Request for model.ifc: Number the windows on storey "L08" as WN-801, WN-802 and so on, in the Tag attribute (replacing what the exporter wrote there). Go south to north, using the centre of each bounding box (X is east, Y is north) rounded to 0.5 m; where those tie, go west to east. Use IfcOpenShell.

First a look at what the model holds.

```python
import ifcopenshell
import ifcopenshell.util.element
import ifcopenshell.util.placement

model = ifcopenshell.open("model.ifc")
print(model.schema)
storey = next(s for s in model.by_type("IfcBuildingStorey") if s.Name == "L08")
windows = [e for e in ifcopenshell.util.element.get_decomposition(storey) if e.is_a("IfcWindow")]
for e in sorted(windows, key=lambda e: e.id()):
    origin = ifcopenshell.util.placement.get_local_placement(e.ObjectPlacement)[:3, 3]
    print(e.id(), e.Tag, e.Name, origin.round(2) + 0.0, sep=" | ")
```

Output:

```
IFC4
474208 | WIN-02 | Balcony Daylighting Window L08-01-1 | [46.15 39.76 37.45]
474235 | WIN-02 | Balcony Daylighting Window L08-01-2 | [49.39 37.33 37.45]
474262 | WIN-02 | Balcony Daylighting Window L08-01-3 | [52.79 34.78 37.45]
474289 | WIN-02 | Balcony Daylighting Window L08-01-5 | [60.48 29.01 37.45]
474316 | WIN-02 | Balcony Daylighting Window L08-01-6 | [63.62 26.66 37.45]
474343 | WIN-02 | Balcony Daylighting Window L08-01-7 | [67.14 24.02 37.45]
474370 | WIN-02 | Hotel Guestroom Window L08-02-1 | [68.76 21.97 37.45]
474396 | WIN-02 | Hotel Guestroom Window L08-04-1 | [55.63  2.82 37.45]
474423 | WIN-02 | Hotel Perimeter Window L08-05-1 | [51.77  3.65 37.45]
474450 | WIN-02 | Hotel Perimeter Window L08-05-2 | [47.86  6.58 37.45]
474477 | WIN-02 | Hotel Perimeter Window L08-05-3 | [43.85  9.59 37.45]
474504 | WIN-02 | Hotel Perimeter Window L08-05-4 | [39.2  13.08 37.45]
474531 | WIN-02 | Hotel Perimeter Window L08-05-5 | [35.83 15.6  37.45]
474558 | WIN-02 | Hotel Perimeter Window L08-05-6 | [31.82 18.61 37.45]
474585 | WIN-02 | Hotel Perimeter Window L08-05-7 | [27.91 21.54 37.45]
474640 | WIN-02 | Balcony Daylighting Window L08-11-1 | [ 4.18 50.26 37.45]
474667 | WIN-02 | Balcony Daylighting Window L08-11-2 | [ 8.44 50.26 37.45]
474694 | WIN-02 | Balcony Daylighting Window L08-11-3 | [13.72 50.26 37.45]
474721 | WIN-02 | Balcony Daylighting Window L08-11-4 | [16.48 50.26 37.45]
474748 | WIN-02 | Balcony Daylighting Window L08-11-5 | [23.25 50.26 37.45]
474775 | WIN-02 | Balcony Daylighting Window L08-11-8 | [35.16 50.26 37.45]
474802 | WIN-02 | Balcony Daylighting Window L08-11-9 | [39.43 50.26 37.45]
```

```python
import ifcopenshell
import ifcopenshell.geom
import ifcopenshell.util.element
import ifcopenshell.util.shape

model = ifcopenshell.open("model.ifc")
settings = ifcopenshell.geom.settings()
settings.set("use-world-coords", True)


def centre(element):
    shape = ifcopenshell.geom.create_shape(settings, element)
    return ifcopenshell.util.shape.get_bbox_centroid(shape.geometry)


storey = next(s for s in model.by_type("IfcBuildingStorey") if s.Name == "L08")
windows = [e for e in ifcopenshell.util.element.get_decomposition(storey) if e.is_a("IfcWindow")]

# Insertion points can sit at a corner or the storey origin, so sort by the geometry (in metres).
centres = {e: centre(e) for e in windows}
windows.sort(key=lambda e: (round(centres[e][1] / 0.5), centres[e][0]))

for i, e in enumerate(windows, start=1):
    number = f"WN-8{i:02d}"
    e.Tag = number
    print(e.id(), number)

model.write("model-out.ifc")
```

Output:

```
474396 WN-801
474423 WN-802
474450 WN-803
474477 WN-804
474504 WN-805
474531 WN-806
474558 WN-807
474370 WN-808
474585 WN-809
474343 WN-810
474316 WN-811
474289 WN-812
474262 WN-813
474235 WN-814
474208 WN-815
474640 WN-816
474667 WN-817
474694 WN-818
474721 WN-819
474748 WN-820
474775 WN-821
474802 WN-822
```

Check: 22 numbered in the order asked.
